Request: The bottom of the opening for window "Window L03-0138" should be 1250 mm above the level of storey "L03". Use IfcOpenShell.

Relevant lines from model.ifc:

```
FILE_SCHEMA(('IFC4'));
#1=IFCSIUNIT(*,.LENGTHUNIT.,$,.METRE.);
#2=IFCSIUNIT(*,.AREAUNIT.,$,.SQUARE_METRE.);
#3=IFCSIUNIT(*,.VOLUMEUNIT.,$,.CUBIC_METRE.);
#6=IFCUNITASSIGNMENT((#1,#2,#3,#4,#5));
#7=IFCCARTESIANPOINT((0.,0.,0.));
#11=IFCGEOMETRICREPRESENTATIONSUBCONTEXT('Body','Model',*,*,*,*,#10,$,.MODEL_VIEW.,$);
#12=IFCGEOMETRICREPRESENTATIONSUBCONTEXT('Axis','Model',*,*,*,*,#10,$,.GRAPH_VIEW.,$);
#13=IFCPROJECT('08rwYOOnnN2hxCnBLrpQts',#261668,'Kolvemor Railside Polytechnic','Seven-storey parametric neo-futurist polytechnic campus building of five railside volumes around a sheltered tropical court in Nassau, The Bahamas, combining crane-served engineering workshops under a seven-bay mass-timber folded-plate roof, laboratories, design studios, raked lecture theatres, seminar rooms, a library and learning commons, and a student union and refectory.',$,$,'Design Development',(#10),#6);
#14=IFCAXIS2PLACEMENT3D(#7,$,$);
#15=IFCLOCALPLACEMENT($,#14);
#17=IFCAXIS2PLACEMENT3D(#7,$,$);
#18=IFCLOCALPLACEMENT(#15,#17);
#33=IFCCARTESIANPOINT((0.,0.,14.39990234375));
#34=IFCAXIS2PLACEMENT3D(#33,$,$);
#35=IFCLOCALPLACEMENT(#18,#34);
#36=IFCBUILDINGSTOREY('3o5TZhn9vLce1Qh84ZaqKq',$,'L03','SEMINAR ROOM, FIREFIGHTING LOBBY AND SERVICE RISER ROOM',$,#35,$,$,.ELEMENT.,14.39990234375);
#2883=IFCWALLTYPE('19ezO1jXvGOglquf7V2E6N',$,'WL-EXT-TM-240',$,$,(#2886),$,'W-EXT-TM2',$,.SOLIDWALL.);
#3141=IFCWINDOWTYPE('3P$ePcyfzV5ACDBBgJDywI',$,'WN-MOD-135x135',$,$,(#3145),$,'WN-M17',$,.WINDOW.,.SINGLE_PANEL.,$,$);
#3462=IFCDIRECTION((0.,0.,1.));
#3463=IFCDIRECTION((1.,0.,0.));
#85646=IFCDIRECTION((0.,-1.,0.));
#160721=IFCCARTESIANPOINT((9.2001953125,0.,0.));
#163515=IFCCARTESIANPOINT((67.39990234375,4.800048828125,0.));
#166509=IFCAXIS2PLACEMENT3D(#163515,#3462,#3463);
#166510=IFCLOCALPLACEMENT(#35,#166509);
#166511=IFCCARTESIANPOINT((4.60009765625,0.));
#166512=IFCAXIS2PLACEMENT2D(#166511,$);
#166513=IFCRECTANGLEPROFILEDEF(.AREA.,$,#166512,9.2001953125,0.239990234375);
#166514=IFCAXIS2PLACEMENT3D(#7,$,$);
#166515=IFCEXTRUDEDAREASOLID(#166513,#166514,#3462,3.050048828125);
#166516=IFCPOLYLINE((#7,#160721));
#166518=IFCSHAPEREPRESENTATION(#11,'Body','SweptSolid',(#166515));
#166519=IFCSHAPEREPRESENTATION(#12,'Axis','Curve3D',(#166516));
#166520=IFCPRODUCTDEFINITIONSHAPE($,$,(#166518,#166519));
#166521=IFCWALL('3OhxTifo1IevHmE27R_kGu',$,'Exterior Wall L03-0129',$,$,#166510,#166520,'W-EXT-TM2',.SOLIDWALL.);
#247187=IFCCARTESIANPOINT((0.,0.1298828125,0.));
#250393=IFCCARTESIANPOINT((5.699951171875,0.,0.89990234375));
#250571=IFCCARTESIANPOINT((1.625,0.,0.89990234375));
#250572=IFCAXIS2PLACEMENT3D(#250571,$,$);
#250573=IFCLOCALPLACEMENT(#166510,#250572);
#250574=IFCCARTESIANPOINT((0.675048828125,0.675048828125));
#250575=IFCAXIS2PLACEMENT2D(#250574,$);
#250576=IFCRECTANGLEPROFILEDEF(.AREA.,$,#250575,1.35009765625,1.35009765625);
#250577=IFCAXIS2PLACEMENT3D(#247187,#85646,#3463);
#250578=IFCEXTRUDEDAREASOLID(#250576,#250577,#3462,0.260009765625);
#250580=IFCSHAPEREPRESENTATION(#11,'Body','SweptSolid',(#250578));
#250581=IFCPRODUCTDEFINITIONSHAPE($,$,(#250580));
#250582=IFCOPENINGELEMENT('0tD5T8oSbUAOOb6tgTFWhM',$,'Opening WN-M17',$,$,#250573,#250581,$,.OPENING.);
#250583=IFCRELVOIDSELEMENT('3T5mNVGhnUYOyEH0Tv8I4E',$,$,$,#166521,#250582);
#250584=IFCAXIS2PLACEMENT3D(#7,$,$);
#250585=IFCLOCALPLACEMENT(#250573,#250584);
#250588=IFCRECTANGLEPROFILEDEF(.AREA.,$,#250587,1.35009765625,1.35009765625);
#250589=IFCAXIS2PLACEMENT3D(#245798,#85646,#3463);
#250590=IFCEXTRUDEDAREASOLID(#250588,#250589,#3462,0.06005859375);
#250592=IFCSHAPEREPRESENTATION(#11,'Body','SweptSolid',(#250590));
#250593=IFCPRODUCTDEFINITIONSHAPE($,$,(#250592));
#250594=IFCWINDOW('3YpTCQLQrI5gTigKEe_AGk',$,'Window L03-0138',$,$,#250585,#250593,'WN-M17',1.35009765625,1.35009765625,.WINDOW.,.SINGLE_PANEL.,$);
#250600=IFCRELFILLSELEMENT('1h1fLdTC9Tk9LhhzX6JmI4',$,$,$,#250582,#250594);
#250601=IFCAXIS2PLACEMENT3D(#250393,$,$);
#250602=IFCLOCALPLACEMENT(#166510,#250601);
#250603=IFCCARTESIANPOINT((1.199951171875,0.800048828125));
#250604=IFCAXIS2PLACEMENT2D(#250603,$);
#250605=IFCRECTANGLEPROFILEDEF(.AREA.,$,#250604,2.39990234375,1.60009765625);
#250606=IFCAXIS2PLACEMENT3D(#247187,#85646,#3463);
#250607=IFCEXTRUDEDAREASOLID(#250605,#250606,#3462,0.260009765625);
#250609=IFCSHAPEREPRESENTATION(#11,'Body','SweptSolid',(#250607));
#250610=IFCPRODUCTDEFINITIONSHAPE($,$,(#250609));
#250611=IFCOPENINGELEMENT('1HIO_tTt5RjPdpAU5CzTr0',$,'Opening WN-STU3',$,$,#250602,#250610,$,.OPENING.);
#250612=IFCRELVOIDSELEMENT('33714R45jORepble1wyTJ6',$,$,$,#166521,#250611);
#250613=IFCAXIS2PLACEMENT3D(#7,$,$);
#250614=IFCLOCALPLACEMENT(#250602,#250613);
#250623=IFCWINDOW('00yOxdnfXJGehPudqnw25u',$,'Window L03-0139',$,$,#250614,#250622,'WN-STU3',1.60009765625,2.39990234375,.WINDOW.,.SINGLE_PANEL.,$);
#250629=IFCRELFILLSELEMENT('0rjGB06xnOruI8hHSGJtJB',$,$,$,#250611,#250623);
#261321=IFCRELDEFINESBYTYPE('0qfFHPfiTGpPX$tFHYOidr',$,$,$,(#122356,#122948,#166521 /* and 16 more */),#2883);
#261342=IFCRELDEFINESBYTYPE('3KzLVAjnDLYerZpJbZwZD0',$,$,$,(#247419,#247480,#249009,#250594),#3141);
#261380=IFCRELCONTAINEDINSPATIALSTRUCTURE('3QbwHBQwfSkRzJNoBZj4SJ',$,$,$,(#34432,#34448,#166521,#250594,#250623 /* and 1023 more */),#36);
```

```python
import numpy as np
import ifcopenshell
import ifcopenshell.api.geometry
import ifcopenshell.geom
import ifcopenshell.util.element
import ifcopenshell.util.placement
import ifcopenshell.util.shape
import ifcopenshell.util.unit

model = ifcopenshell.open("model.ifc")
unit_scale = ifcopenshell.util.unit.calculate_unit_scale(model)

window = model.by_guid("3YpTCQLQrI5gTigKEe_AGk")
opening = window.FillsVoids[0].RelatingOpeningElement
storey = ifcopenshell.util.element.get_container(window, ifc_class="IfcBuildingStorey")
level = ifcopenshell.util.placement.get_local_placement(storey.ObjectPlacement)[2, 3]

# The opening's origin need not be at the sill, so measure its lowest point.
shape = ifcopenshell.geom.create_shape(ifcopenshell.geom.settings(), opening)
bottom = ifcopenshell.util.shape.get_shape_bottom_elevation(shape, shape.geometry) / unit_scale
dz = level + 1.25 / unit_scale - bottom

shift = np.array([0.0, 0.0, dz])
# The window is placed relative to its opening, so it follows when the opening moves.
matrix = ifcopenshell.util.placement.get_local_placement(opening.ObjectPlacement)
matrix[:3, 3] += shift
ifcopenshell.api.geometry.edit_object_placement(
    model, product=opening, matrix=matrix, is_si=False, should_transform_children=True
)

print(f"moved by {dz * unit_scale:+.3f} m")

model.write("model_updated.ifc")
```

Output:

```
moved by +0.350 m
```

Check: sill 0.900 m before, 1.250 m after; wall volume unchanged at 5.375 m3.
